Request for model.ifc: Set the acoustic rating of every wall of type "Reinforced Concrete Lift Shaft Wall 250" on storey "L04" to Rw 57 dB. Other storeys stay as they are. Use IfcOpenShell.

First a look at what the model holds.

```python
import ifcopenshell
import ifcopenshell.util.element

model = ifcopenshell.open("model.ifc")
print(model.schema)
storey = next(s for s in model.by_type("IfcBuildingStorey") if s.Name == "L04")
walls = [e for e in ifcopenshell.util.element.get_decomposition(storey) if e.is_a("IfcWall")]
seen = {}
for e in walls:
    element_type = ifcopenshell.util.element.get_type(e)
    key = (element_type.Name if element_type != e and element_type else None, ifcopenshell.util.element.get_pset(e, "Pset_WallCommon", "AcousticRating"))
    seen[key] = seen.get(key, 0) + 1
for (name, value), count in sorted(seen.items(), key=str):
    print(count, "x", name, "|", value)
```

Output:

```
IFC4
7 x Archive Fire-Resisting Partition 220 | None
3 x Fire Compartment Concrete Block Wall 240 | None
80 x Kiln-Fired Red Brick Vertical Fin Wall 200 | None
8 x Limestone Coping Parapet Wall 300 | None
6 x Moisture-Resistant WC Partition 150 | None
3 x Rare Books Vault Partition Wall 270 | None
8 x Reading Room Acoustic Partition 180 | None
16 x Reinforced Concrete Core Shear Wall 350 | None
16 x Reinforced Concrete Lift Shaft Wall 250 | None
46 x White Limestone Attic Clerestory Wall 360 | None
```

```python
import ifcopenshell
import ifcopenshell.api.pset
import ifcopenshell.util.element

model = ifcopenshell.open("model.ifc")

storey = next(s for s in model.by_type("IfcBuildingStorey") if s.Name == "L04")
walls = [e for e in ifcopenshell.util.element.get_decomposition(storey) if e.is_a("IfcWall")]

count = 0
for e in walls:
    element_type = ifcopenshell.util.element.get_type(e)
    if element_type in (None, e) or element_type.Name != "Reinforced Concrete Lift Shaft Wall 250":
        continue
    # add_pset returns the element's existing set when there is one.
    pset = ifcopenshell.api.pset.add_pset(model, product=e, name="Pset_WallCommon")
    ifcopenshell.api.pset.edit_pset(model, pset=pset, properties={"AcousticRating": "Rw 57 dB"})
    count += 1

print(count, "walls updated")

model.write("model-out.ifc")
```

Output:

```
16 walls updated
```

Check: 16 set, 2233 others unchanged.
